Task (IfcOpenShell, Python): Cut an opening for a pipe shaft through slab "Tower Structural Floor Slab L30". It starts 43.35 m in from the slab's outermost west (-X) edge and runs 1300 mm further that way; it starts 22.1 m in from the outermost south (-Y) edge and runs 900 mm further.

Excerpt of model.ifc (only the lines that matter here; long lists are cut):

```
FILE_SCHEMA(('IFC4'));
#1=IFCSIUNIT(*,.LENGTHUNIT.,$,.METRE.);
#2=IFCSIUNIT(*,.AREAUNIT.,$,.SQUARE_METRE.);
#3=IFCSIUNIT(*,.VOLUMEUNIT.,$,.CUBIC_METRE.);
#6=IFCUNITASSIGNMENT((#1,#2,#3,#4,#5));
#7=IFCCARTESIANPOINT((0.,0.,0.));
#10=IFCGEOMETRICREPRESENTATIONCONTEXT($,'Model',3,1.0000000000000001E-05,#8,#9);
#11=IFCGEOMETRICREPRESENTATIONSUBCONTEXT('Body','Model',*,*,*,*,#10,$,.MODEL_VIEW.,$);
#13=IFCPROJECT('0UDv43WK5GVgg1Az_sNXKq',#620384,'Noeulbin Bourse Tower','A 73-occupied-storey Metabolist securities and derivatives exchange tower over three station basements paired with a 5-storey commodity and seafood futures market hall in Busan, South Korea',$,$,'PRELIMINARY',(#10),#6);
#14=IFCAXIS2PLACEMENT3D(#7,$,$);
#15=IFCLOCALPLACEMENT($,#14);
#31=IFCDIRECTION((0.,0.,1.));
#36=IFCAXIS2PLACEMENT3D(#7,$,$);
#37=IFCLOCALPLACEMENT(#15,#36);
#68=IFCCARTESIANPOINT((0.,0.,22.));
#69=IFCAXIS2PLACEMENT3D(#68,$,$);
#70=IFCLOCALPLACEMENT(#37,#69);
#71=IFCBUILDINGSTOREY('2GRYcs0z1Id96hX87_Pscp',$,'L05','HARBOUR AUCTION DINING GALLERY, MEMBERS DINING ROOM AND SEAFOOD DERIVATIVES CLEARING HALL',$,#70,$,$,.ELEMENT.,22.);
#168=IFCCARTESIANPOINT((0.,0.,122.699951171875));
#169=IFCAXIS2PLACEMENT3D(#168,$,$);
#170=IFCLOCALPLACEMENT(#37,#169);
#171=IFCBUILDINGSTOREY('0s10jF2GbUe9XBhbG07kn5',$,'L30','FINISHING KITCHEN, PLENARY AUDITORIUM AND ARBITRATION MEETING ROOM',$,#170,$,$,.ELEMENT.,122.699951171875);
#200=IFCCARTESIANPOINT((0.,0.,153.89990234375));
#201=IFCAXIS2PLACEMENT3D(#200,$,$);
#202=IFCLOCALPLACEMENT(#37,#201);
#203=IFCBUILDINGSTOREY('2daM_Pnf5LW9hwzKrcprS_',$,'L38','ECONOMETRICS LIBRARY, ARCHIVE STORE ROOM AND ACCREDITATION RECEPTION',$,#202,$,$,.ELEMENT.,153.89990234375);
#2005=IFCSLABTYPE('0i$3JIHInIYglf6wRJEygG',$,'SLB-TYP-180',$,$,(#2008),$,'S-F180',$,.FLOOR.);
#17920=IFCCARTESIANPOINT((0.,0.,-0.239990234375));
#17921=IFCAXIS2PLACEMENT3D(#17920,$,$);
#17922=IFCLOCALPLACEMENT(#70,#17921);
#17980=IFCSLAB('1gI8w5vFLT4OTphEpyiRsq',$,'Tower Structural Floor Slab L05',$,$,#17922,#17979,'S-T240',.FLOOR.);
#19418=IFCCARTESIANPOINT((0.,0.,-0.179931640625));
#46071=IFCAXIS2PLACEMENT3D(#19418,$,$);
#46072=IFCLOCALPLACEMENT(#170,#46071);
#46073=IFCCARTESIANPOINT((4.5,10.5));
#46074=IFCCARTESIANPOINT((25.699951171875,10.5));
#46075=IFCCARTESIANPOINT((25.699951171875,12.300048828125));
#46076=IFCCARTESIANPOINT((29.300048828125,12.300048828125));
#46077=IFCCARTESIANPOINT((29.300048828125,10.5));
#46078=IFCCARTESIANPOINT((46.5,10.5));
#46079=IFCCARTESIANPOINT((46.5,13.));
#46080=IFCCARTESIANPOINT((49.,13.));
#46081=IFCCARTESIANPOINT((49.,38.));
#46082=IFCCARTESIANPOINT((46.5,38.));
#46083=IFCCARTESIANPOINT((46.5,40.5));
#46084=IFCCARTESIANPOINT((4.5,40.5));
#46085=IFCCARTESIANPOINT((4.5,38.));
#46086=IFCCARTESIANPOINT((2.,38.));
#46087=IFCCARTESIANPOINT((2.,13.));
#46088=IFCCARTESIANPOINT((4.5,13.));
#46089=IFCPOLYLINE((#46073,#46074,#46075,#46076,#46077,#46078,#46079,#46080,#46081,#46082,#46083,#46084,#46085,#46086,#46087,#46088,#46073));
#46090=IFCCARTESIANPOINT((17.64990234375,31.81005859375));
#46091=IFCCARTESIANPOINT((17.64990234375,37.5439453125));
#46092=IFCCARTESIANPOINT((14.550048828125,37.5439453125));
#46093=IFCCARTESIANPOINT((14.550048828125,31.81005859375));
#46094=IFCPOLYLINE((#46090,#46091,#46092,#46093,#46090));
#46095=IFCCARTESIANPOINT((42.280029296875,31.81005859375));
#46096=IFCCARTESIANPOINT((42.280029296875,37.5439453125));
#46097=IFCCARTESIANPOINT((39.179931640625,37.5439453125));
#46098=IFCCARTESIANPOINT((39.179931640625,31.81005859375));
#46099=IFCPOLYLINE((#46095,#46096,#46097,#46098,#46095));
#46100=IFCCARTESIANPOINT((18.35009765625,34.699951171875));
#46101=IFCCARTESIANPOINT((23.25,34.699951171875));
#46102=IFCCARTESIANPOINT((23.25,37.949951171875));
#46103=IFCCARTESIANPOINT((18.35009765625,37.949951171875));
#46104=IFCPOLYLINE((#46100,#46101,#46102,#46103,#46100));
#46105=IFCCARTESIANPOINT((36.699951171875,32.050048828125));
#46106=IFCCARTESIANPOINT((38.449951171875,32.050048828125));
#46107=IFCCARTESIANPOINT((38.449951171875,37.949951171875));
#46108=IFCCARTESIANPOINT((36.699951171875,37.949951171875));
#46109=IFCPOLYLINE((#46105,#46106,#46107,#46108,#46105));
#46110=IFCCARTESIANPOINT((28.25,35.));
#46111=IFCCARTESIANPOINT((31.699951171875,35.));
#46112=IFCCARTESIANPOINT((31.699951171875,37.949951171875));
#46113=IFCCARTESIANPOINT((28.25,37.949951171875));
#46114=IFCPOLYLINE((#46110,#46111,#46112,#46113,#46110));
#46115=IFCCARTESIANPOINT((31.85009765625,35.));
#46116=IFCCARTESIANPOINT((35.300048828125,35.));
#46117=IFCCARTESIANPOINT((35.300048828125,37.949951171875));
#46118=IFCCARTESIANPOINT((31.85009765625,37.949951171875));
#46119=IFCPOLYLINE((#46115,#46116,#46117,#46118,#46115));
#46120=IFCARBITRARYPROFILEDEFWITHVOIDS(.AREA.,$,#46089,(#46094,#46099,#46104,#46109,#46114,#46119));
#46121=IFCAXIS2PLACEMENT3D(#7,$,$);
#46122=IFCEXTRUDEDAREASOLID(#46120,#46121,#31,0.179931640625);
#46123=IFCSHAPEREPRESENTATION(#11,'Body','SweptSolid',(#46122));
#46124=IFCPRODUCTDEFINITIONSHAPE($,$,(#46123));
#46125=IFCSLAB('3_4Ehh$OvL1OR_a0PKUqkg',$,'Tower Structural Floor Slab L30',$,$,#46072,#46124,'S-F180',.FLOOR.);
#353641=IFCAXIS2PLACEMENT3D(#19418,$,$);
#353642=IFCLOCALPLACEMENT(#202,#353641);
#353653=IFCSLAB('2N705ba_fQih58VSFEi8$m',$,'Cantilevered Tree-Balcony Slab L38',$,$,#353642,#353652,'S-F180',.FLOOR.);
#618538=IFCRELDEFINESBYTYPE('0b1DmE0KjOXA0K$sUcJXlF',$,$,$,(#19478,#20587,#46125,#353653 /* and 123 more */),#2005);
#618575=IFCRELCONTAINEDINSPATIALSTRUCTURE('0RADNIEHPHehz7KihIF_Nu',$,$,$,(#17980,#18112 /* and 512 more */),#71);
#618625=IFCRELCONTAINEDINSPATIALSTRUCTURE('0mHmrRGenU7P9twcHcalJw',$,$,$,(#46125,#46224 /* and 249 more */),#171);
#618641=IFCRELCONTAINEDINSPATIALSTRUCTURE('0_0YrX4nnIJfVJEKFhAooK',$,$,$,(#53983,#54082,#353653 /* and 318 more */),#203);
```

```python
import numpy as np
import ifcopenshell
import ifcopenshell.api.feature
import ifcopenshell.api.geometry
import ifcopenshell.api.root
import ifcopenshell.geom
import ifcopenshell.util.placement
import ifcopenshell.util.representation
import ifcopenshell.util.shape
import ifcopenshell.util.unit

model = ifcopenshell.open("model.ifc")
unit_scale = ifcopenshell.util.unit.calculate_unit_scale(model)
settings = ifcopenshell.geom.settings()


def volume(element):
    """Net volume in cubic metres, openings subtracted."""
    shape = ifcopenshell.geom.create_shape(settings, element)
    return ifcopenshell.util.shape.get_volume(shape.geometry)


slab = model.by_guid("3_4Ehh$OvL1OR_a0PKUqkg")
before = volume(slab)

# Extent in the slab's own axes, in metres. The edges named are its -X and -Y sides.
slab_shape = ifcopenshell.geom.create_shape(settings, slab)
vertices = ifcopenshell.util.shape.get_vertices(slab_shape.geometry)
x_min, y_min, bottom = vertices.min(axis=0)
top = vertices[:, 2].max()

opening = ifcopenshell.api.root.create_entity(model, ifc_class="IfcOpeningElement", name="Pipe shaft opening", predefined_type="OPENING")
context = ifcopenshell.util.representation.get_context(model, "Model", "Body", "MODEL_VIEW")
width, depth = 1.3, 0.9
outline = [(0.0, 0.0), (width, 0.0), (width, depth), (0.0, depth), (0.0, 0.0)]
# Overshoot both faces by 50 mm so the cut is clean.
shape = ifcopenshell.api.geometry.add_slab_representation(
    model, context=context, depth=top - bottom + 0.1, polyline=outline
)
ifcopenshell.api.geometry.assign_representation(model, product=opening, representation=shape)

matrix = ifcopenshell.util.placement.get_local_placement(slab.ObjectPlacement)
matrix[:, 3] = matrix @ np.append(np.array([x_min + 43.35, y_min + 22.1, bottom - 0.05]) / unit_scale, 1.0)
ifcopenshell.api.geometry.edit_object_placement(model, product=opening, matrix=matrix, is_si=False)
ifcopenshell.api.feature.add_feature(model, feature=opening, element=slab)

after = volume(slab)

print(f"slab volume {before:.3f} -> {after:.3f} m3")

model.write("model_v2.ifc")
```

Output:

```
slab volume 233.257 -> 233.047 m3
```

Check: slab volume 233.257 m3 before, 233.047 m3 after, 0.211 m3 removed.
